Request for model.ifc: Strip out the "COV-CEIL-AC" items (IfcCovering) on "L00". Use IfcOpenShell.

First a look at what the model holds.

```python
import ifcopenshell
import ifcopenshell.util.element

model = ifcopenshell.open("model.ifc")
print(model.schema)
storey = next(s for s in model.by_type("IfcBuildingStorey") if s.Name == "L00")
coverings = [e for e in ifcopenshell.util.element.get_decomposition(storey) if e.is_a("IfcCovering")]
seen = {}
for e in coverings:
    element_type = ifcopenshell.util.element.get_type(e)
    name = element_type.Name if element_type not in (None, e) else None
    seen[name] = seen.get(name, 0) + 1
for name, count in sorted(seen.items(), key=str):
    print(count, "x", name)
```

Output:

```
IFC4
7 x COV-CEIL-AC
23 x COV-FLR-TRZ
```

```python
import ifcopenshell
import ifcopenshell.api.root
import ifcopenshell.util.element

model = ifcopenshell.open("model.ifc")

storey = next(s for s in model.by_type("IfcBuildingStorey") if s.Name == "L00")
coverings = [e for e in ifcopenshell.util.element.get_decomposition(storey) if e.is_a("IfcCovering")]
targets = [e for e in coverings if (t := ifcopenshell.util.element.get_type(e)) not in (None, e) and t.Name == "COV-CEIL-AC"]

for e in targets:
    ifcopenshell.api.root.remove_product(model, product=e)
print(len(targets), "removed")

model.write("model_rev.ifc")
```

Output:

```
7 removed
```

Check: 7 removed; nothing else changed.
